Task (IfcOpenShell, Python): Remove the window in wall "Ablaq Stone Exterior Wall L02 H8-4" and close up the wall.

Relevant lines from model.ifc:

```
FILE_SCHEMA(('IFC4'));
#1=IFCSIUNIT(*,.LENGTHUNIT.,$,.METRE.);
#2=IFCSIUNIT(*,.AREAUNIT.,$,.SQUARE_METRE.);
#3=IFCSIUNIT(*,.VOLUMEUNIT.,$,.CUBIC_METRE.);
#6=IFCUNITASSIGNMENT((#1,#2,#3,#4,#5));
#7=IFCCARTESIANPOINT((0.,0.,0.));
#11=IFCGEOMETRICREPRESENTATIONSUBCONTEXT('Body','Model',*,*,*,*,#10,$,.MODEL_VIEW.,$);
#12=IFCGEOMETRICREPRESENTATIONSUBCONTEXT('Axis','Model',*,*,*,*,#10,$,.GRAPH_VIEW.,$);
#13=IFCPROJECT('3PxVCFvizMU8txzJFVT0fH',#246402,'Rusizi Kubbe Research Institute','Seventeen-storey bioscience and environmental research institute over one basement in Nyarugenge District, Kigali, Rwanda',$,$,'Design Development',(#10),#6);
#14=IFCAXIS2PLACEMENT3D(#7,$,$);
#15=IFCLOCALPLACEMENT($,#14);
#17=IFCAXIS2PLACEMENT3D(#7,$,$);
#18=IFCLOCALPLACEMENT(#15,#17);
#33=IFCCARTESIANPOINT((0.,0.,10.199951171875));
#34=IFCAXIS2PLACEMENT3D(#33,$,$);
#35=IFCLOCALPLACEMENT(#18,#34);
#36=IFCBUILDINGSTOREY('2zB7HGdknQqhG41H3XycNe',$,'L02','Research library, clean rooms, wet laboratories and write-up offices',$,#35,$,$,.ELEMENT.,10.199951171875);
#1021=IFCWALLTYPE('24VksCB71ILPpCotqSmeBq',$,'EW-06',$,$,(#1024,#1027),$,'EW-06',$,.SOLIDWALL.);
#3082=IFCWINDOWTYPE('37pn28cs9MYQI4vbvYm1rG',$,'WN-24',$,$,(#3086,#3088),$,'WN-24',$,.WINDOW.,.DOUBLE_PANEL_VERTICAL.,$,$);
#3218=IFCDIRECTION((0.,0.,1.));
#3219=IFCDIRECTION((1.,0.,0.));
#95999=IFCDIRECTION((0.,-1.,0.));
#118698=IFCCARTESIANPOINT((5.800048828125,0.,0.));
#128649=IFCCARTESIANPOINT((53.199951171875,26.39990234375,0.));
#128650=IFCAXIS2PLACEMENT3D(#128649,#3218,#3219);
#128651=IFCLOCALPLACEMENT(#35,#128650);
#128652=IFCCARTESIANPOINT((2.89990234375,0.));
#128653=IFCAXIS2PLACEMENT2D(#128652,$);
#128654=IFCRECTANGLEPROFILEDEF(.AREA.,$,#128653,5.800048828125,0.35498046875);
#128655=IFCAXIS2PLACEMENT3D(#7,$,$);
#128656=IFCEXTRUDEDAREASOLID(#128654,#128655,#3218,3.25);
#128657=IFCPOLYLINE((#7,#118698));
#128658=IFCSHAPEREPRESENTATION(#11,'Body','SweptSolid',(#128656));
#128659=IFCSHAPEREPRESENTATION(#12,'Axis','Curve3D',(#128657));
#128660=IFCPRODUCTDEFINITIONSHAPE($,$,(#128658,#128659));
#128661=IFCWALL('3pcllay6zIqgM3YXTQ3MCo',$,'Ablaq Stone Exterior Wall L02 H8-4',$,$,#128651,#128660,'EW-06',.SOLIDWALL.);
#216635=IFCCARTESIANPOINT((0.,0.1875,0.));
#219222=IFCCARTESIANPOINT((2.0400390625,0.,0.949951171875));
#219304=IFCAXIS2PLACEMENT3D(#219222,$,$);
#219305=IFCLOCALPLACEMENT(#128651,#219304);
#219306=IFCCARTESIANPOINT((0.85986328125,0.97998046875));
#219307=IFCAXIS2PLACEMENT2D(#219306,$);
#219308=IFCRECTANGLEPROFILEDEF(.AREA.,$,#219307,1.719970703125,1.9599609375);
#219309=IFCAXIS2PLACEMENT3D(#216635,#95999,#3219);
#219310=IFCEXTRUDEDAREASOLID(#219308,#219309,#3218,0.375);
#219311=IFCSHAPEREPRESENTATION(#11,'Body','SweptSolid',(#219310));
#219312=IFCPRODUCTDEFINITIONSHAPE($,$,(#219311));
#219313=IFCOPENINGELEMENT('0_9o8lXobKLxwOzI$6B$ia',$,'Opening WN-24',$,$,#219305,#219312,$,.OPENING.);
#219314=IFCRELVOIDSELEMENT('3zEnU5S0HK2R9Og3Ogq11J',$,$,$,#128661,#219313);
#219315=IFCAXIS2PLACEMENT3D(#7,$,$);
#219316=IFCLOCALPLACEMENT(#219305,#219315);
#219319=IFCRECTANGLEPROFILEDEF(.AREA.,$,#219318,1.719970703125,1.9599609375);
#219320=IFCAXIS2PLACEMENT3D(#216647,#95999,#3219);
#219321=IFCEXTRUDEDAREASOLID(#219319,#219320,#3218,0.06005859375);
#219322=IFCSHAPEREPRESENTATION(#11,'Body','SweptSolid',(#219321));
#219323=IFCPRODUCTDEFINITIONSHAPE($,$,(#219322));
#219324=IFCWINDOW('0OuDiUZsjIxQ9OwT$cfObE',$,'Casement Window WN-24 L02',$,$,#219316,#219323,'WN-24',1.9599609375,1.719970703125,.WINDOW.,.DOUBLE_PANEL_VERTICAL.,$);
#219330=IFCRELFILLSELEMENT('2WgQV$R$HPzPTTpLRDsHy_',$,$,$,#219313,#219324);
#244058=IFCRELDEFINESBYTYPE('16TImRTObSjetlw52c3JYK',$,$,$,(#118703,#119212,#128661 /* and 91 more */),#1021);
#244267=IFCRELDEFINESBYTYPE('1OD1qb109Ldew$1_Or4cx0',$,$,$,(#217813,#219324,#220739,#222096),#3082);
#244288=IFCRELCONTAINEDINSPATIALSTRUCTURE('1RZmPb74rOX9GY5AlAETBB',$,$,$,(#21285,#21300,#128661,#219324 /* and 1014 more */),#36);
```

```python
import ifcopenshell
import ifcopenshell.api.feature
import ifcopenshell.api.root
import ifcopenshell.geom
import ifcopenshell.util.shape

model = ifcopenshell.open("model.ifc")
settings = ifcopenshell.geom.settings()


def volume(element):
    """Net volume in cubic metres, openings subtracted."""
    shape = ifcopenshell.geom.create_shape(settings, element)
    return ifcopenshell.util.shape.get_volume(shape.geometry)


window = model.by_guid("0OuDiUZsjIxQ9OwT$cfObE")
opening = window.FillsVoids[0].RelatingOpeningElement
wall = opening.VoidsElements[0].RelatingBuildingElement
before = volume(wall)

ifcopenshell.api.root.remove_product(model, product=window)
ifcopenshell.api.feature.remove_feature(model, feature=opening)

after = volume(wall)

print(f"wall volume {before:.3f} -> {after:.3f} m3")

model.write("model_edited.ifc")
```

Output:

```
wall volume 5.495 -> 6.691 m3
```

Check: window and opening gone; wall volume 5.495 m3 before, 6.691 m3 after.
